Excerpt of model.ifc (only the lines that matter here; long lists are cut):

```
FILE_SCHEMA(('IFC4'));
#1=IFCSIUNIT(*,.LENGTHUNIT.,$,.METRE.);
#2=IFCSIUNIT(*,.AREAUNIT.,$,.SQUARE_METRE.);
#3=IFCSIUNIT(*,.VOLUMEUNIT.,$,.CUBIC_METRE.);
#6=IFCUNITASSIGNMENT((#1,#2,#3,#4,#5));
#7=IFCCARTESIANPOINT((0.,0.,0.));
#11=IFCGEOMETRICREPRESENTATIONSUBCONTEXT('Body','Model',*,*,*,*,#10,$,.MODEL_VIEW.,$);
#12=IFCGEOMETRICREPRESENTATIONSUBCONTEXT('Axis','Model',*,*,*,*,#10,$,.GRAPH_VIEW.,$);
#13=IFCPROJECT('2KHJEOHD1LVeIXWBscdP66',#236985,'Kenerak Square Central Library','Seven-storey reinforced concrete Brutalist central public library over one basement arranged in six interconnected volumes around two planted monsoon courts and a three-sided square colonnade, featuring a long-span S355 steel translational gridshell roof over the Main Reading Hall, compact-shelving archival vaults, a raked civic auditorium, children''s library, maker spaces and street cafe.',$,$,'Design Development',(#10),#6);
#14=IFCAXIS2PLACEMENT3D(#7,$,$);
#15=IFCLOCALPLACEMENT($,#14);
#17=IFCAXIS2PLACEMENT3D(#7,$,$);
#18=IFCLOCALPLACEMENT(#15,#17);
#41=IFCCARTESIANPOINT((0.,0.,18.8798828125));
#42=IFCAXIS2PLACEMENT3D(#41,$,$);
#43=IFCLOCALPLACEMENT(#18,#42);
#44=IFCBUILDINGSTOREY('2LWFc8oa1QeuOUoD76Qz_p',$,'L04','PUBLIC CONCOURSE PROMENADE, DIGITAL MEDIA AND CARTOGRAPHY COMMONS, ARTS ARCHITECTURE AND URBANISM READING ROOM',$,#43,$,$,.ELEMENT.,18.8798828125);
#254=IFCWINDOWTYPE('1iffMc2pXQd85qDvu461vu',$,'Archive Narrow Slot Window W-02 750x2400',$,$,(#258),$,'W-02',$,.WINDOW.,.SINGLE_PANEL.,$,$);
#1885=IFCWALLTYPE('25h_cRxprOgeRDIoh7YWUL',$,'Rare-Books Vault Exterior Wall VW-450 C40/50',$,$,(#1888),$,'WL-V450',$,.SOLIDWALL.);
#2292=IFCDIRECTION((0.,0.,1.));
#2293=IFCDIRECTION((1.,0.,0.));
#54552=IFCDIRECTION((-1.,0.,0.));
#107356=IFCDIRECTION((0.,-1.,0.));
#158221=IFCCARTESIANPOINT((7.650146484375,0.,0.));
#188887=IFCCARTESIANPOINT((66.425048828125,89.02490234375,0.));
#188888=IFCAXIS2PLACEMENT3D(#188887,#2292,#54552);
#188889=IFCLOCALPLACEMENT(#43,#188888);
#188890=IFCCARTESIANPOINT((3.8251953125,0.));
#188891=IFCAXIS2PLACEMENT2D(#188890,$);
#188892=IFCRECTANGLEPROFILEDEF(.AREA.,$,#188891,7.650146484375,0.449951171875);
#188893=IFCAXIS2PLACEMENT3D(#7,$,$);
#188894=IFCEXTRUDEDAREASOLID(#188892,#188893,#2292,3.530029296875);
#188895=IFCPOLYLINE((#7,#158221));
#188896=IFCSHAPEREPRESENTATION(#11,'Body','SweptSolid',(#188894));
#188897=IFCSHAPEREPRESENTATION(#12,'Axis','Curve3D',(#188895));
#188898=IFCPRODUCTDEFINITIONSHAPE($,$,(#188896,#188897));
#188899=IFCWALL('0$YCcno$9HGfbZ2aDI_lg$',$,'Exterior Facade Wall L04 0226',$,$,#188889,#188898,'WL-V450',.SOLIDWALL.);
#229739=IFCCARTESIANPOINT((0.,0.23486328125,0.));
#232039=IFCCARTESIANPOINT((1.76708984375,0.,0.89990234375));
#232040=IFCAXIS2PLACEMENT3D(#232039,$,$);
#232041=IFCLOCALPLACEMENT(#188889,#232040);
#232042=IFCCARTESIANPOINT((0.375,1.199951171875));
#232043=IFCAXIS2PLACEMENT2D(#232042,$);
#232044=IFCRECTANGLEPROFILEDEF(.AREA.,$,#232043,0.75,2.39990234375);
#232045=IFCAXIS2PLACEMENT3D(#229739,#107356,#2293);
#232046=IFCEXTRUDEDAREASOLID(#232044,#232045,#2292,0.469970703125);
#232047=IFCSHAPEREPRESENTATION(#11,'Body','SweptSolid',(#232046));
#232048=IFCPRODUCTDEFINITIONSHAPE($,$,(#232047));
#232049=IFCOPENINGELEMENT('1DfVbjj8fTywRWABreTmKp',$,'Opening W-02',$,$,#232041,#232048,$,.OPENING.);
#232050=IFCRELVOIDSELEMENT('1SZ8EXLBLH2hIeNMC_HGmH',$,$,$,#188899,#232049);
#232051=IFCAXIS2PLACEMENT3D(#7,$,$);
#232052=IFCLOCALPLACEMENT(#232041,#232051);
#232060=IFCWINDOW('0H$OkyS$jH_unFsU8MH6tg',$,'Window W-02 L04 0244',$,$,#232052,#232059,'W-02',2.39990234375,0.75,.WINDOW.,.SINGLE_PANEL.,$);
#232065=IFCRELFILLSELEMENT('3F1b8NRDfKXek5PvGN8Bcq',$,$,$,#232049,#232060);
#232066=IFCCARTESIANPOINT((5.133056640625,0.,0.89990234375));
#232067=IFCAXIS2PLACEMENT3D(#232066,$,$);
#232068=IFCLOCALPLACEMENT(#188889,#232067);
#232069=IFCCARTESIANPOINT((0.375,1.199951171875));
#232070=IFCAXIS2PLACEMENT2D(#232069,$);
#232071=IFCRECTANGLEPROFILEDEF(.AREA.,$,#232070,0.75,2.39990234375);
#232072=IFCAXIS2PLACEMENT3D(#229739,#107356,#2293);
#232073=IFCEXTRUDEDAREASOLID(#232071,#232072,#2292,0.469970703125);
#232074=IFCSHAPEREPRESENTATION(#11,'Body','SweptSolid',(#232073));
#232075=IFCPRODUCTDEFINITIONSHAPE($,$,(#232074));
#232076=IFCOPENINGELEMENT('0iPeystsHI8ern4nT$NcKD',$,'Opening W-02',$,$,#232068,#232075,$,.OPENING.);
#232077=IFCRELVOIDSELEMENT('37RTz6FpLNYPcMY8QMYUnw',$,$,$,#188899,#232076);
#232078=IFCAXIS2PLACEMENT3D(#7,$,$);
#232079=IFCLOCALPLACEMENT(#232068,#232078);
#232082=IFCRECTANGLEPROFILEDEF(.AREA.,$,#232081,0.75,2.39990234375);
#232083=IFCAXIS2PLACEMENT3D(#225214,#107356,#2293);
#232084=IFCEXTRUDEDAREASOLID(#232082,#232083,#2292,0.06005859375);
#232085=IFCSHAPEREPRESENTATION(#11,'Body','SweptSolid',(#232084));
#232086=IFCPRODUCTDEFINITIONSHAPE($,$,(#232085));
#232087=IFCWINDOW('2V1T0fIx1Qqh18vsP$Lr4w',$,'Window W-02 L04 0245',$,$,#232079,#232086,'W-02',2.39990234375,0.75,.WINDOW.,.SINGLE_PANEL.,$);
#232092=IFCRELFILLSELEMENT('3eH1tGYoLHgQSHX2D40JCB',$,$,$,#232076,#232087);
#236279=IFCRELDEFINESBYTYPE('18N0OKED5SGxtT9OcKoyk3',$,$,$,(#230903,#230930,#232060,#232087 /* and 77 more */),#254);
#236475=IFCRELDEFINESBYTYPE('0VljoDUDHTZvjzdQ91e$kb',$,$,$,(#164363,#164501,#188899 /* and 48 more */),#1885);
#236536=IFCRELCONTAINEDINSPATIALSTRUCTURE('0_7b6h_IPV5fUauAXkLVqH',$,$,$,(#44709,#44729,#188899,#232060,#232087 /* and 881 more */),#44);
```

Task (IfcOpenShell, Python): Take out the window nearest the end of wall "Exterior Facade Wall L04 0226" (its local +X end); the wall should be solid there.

```python
import ifcopenshell
import ifcopenshell.api.feature
import ifcopenshell.api.root
import ifcopenshell.geom
import ifcopenshell.util.shape

model = ifcopenshell.open("model.ifc")
settings = ifcopenshell.geom.settings()


def volume(element):
    """Net volume in cubic metres, openings subtracted."""
    shape = ifcopenshell.geom.create_shape(settings, element)
    return ifcopenshell.util.shape.get_volume(shape.geometry)


window = model.by_guid("2V1T0fIx1Qqh18vsP$Lr4w")
opening = window.FillsVoids[0].RelatingOpeningElement
wall = opening.VoidsElements[0].RelatingBuildingElement
before = volume(wall)

ifcopenshell.api.root.remove_product(model, product=window)
ifcopenshell.api.feature.remove_feature(model, feature=opening)

after = volume(wall)

print(f"wall volume {before:.3f} -> {after:.3f} m3")

model.write("model_updated.ifc")
```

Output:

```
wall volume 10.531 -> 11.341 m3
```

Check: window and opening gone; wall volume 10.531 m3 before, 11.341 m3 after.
